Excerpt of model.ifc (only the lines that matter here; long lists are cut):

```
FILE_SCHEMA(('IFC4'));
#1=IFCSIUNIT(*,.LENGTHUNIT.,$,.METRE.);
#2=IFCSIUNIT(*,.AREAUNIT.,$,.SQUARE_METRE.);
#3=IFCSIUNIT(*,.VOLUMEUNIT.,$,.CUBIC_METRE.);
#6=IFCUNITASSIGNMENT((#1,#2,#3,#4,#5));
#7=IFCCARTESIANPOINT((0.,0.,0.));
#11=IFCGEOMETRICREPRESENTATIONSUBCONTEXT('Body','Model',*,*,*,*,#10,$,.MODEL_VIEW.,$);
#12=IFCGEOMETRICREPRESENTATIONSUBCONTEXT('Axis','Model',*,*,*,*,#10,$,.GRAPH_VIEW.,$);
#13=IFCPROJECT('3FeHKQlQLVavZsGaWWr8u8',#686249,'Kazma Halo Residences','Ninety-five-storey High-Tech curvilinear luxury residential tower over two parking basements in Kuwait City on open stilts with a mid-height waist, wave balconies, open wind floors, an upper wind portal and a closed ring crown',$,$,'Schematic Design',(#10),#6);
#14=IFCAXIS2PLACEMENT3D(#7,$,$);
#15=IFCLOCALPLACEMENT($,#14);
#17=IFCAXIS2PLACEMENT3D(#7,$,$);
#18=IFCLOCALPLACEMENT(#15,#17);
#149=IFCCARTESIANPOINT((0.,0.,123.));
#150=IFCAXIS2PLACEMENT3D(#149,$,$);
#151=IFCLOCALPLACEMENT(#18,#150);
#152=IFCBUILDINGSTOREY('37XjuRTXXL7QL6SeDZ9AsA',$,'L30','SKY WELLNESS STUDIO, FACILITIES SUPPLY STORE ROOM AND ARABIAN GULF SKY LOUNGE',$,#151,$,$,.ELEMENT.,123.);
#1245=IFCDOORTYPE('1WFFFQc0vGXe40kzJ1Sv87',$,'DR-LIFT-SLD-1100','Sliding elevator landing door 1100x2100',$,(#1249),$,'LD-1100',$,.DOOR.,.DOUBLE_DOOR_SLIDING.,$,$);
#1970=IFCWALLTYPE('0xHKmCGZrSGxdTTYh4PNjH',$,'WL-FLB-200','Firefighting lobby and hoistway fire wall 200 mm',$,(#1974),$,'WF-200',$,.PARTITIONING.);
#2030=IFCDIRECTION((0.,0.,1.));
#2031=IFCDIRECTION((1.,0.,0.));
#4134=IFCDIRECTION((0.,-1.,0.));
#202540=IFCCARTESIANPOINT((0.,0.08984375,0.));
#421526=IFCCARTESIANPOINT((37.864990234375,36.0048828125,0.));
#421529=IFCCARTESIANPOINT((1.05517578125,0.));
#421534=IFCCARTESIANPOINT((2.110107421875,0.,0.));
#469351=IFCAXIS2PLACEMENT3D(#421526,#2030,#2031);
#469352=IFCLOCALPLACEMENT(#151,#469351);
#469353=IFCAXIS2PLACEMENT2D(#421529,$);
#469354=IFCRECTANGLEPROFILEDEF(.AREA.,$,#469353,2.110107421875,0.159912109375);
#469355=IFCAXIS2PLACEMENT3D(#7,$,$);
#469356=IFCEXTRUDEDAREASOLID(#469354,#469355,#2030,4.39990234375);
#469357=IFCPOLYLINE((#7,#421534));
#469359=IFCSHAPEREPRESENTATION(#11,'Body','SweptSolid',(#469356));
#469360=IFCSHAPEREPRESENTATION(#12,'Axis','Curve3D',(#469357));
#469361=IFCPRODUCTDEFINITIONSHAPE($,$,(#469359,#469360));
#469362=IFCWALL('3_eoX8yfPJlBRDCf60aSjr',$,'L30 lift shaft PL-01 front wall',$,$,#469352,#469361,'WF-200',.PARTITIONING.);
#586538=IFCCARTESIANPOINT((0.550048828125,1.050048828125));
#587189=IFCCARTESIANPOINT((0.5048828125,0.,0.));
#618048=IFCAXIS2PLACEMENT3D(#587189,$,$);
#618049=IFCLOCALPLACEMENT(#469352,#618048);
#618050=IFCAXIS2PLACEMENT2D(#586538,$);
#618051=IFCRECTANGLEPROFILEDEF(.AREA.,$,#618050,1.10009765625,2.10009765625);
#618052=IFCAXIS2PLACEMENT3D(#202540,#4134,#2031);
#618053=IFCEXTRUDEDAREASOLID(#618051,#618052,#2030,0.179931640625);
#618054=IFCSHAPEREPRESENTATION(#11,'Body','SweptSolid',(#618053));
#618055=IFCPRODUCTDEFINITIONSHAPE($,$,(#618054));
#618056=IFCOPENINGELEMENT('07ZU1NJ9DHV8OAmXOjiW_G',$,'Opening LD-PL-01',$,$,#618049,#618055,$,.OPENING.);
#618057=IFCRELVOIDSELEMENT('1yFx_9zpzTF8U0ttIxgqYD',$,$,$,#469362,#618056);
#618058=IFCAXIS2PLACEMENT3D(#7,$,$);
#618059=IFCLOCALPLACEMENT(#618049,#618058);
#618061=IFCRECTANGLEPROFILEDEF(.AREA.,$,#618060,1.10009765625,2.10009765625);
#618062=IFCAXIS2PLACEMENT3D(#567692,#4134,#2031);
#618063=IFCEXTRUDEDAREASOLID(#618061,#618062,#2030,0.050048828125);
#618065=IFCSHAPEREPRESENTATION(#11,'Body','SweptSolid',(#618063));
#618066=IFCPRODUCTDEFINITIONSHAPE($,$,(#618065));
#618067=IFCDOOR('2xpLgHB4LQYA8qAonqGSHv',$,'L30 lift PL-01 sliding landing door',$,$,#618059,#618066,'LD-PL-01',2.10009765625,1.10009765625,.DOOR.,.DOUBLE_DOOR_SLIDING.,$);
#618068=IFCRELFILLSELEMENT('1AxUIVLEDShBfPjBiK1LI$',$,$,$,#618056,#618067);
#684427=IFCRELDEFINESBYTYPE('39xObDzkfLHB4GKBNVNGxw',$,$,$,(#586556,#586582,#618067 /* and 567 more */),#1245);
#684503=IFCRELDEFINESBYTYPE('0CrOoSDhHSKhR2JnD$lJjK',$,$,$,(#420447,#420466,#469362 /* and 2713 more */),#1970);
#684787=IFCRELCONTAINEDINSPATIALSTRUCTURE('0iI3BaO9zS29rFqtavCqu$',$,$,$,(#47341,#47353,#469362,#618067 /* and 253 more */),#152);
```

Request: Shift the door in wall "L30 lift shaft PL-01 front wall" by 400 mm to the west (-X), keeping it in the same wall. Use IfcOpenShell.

```python
import ifcopenshell
import ifcopenshell.api.geometry
import ifcopenshell.util.placement
import ifcopenshell.util.unit

model = ifcopenshell.open("model.ifc")
unit_scale = ifcopenshell.util.unit.calculate_unit_scale(model)

door = model.by_id(618067)
opening = door.FillsVoids[0].RelatingOpeningElement
wall = opening.VoidsElements[0].RelatingBuildingElement

wall_matrix = ifcopenshell.util.placement.get_local_placement(wall.ObjectPlacement)
shift = wall_matrix[:3, 0] * -0.4 / unit_scale
before = ifcopenshell.util.placement.get_local_placement(door.ObjectPlacement)[:3, 3].copy()

# The door is placed relative to its opening, so it follows when the opening moves.
matrix = ifcopenshell.util.placement.get_local_placement(opening.ObjectPlacement)
matrix[:3, 3] += shift
ifcopenshell.api.geometry.edit_object_placement(
    model, product=opening, matrix=matrix, is_si=False, should_transform_children=True
)

after = ifcopenshell.util.placement.get_local_placement(door.ObjectPlacement)[:3, 3]
print("door moved by", (after - before).round(3) + 0.0)

model.write("model_edited.ifc")
```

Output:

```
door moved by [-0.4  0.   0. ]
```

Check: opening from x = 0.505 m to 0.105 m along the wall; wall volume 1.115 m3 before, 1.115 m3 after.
